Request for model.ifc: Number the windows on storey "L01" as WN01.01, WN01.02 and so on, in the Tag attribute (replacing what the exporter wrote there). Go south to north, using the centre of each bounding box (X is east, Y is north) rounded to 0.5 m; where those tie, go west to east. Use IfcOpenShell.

First a look at what the model holds.

```python
import ifcopenshell
import ifcopenshell.util.element
import ifcopenshell.util.placement

model = ifcopenshell.open("model.ifc")
print(model.schema)
storey = next(s for s in model.by_type("IfcBuildingStorey") if s.Name == "L01")
windows = [e for e in ifcopenshell.util.element.get_decomposition(storey) if e.is_a("IfcWindow")]
for e in sorted(windows, key=lambda e: e.id()):
    origin = ifcopenshell.util.placement.get_local_placement(e.ObjectPlacement)[:3, 3]
    print(e.id(), e.Tag, e.Name, origin.round(2) + 0.0, sep=" | ")
```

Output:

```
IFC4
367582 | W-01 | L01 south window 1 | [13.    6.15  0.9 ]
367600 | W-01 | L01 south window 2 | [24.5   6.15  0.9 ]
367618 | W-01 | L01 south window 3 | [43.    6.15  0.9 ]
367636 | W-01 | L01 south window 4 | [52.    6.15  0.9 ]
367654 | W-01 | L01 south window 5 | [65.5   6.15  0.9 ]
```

```python
import ifcopenshell
import ifcopenshell.geom
import ifcopenshell.util.element
import ifcopenshell.util.shape

model = ifcopenshell.open("model.ifc")
settings = ifcopenshell.geom.settings()
settings.set("use-world-coords", True)


def centre(element):
    shape = ifcopenshell.geom.create_shape(settings, element)
    return ifcopenshell.util.shape.get_bbox_centroid(shape.geometry)


storey = next(s for s in model.by_type("IfcBuildingStorey") if s.Name == "L01")
windows = [e for e in ifcopenshell.util.element.get_decomposition(storey) if e.is_a("IfcWindow")]

# Insertion points can sit at a corner or the storey origin, so sort by the geometry (in metres).
centres = {e: centre(e) for e in windows}
windows.sort(key=lambda e: (round(centres[e][1] / 0.5), centres[e][0]))

for i, e in enumerate(windows, start=1):
    number = f"WN01.{i:02d}"
    e.Tag = number
    print(e.id(), number)

model.write("model_rev.ifc")
```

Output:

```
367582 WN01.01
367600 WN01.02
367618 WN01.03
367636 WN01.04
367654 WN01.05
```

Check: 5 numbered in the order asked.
